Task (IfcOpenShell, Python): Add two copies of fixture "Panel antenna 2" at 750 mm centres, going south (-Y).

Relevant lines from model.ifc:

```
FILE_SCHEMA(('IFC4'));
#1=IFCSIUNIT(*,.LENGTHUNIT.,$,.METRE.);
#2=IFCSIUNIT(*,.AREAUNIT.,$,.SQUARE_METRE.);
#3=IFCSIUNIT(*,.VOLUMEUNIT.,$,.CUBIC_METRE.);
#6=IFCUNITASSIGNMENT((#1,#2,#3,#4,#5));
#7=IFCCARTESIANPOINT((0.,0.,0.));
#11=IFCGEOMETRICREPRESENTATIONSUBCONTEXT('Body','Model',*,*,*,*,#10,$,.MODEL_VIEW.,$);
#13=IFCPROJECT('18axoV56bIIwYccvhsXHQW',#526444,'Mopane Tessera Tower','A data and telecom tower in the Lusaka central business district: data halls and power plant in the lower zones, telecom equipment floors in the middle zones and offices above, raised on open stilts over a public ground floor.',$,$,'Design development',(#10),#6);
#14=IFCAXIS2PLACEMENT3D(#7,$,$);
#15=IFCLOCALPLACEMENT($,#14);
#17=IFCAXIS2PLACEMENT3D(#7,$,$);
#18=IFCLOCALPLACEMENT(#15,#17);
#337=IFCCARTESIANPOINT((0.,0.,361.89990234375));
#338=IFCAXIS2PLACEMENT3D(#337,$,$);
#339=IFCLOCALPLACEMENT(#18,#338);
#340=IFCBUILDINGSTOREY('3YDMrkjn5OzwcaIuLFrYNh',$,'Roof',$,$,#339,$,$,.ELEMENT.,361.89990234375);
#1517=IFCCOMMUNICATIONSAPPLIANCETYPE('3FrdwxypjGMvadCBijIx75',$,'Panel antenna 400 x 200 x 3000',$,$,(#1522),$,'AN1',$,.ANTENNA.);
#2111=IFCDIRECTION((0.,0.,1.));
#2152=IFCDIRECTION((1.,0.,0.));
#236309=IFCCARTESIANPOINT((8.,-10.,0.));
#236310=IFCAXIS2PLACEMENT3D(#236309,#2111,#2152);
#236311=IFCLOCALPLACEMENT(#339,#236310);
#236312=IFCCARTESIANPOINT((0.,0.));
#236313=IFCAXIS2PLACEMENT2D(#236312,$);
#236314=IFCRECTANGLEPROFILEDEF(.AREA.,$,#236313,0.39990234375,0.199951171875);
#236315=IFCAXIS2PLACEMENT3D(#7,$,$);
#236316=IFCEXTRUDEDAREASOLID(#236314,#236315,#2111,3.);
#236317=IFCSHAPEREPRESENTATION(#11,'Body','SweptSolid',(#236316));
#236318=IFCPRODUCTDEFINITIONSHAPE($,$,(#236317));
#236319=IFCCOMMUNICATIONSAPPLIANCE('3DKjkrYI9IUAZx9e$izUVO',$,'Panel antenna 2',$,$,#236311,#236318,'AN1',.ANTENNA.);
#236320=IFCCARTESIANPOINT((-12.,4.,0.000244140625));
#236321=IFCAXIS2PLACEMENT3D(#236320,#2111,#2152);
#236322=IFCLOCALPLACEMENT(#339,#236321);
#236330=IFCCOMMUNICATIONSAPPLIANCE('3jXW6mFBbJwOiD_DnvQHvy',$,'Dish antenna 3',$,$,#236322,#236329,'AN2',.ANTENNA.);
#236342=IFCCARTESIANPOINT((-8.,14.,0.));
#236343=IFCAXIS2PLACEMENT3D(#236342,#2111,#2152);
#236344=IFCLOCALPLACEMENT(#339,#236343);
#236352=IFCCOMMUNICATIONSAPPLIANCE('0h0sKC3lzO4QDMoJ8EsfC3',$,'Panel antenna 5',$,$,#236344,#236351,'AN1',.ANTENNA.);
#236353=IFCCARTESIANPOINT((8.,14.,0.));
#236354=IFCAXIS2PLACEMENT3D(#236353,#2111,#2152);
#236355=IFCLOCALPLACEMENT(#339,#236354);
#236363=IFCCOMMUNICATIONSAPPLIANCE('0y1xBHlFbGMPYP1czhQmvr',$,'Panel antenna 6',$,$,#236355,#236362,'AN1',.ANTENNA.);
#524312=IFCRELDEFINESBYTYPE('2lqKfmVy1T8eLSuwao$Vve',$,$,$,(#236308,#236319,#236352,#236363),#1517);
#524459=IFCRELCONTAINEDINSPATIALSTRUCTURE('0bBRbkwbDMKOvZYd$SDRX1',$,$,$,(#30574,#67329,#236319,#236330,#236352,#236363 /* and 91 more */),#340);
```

```python
import numpy as np
import ifcopenshell
import ifcopenshell.api.geometry
import ifcopenshell.api.root
import ifcopenshell.util.element
import ifcopenshell.util.placement
import ifcopenshell.util.unit

model = ifcopenshell.open("model.ifc")
unit_scale = ifcopenshell.util.unit.calculate_unit_scale(model)

source = model.by_id(236319)
base = ifcopenshell.util.placement.get_local_placement(source.ObjectPlacement)
step = np.array([0.0, -1.0, 0.0]) * 0.75 / unit_scale

for i in range(1, 3):
    copy = ifcopenshell.api.root.copy_class(model, product=source)
    copy.Representation = ifcopenshell.util.element.copy_deep(
        model, source.Representation, exclude=["IfcGeometricRepresentationContext", "IfcRepresentationMap"]
    )
    copy.Tag = None
    matrix = base.copy()
    matrix[:3, 3] += i * step
    print("added at", matrix[:3, 3].round(3) + 0.0)
    ifcopenshell.api.geometry.edit_object_placement(model, product=copy, matrix=matrix, is_si=False)

model.write("model_updated.ifc")
```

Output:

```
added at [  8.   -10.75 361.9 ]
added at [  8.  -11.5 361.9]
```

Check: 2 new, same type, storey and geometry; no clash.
